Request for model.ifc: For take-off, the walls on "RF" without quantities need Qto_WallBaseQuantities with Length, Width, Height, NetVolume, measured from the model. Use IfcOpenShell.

First a look at what the model holds.

```python
import ifcopenshell
import ifcopenshell.util.element
import ifcopenshell.util.unit

model = ifcopenshell.open("model.ifc")
print(model.schema)
for unit_type in ("LENGTHUNIT", "AREAUNIT", "VOLUMEUNIT"):
    print(unit_type, ifcopenshell.util.unit.calculate_unit_scale(model, unit_type))
storey = next(s for s in model.by_type("IfcBuildingStorey") if s.Name == "RF")
walls = [e for e in ifcopenshell.util.element.get_decomposition(storey) if e.is_a("IfcWall")]
for e in sorted(walls, key=lambda e: e.id()):
    print(e.id(), e.is_a(), e.Name, list(ifcopenshell.util.element.get_psets(e, qtos_only=True)), sep=" | ")
```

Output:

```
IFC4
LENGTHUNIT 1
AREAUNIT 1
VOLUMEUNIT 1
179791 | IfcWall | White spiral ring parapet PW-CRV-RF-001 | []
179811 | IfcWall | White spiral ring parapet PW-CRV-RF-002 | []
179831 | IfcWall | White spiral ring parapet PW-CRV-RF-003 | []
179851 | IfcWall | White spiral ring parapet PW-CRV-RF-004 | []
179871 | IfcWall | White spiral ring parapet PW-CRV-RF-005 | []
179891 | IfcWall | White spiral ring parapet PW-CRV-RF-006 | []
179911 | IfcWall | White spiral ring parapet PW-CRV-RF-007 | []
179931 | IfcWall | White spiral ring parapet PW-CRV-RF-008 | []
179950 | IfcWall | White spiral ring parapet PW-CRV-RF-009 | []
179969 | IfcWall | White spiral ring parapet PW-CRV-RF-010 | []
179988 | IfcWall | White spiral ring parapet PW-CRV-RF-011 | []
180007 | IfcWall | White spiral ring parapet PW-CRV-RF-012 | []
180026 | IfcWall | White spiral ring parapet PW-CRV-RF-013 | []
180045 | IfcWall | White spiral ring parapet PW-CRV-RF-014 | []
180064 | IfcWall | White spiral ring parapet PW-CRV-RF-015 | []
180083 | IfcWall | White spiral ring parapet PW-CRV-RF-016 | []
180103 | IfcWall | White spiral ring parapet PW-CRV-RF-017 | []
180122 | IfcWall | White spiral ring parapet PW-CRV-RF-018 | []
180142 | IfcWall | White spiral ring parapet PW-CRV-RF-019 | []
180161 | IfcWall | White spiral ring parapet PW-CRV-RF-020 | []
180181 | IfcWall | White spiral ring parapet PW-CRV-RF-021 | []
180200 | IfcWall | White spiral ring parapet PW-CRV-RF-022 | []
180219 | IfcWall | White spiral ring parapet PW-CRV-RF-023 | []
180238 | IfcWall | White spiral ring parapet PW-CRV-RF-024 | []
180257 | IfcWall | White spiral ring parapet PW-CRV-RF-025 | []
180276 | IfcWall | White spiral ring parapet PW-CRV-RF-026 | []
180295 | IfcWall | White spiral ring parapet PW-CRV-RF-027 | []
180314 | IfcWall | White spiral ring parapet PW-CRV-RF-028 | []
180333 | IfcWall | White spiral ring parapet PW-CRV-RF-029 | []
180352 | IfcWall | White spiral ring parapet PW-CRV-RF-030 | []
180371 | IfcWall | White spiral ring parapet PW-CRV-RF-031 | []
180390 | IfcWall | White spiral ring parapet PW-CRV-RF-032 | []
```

```python
import ifcopenshell
import ifcopenshell.api.pset
import ifcopenshell.geom
import ifcopenshell.util.element
import ifcopenshell.util.shape
import ifcopenshell.util.unit

model = ifcopenshell.open("model.ifc")
unit_scale = ifcopenshell.util.unit.calculate_unit_scale(model)
volume_scale = ifcopenshell.util.unit.calculate_unit_scale(model, "VOLUMEUNIT")
settings = ifcopenshell.geom.settings()

storey = next(s for s in model.by_type("IfcBuildingStorey") if s.Name == "RF")
walls = [e for e in ifcopenshell.util.element.get_decomposition(storey) if e.is_a("IfcWall")]

for e in sorted(walls, key=lambda e: e.id()):
    if ifcopenshell.util.element.get_psets(e, qtos_only=True, should_inherit=False):
        continue
    # Geometry comes back in metres, in the element's own axes.
    shape = ifcopenshell.geom.create_shape(settings, e)
    values = {
        "Length": ifcopenshell.util.shape.get_x(shape.geometry) / unit_scale,
        "Width": ifcopenshell.util.shape.get_y(shape.geometry) / unit_scale,
        "Height": ifcopenshell.util.shape.get_z(shape.geometry) / unit_scale,
        "NetVolume": ifcopenshell.util.shape.get_volume(shape.geometry) / volume_scale,
    }
    qto = ifcopenshell.api.pset.add_qto(model, product=e, name="Qto_WallBaseQuantities")
    ifcopenshell.api.pset.edit_qto(model, qto=qto, properties=values)
    print(e.id(), {k: round(v, 3) for k, v in values.items()})

model.write("model_rev.ifc")
```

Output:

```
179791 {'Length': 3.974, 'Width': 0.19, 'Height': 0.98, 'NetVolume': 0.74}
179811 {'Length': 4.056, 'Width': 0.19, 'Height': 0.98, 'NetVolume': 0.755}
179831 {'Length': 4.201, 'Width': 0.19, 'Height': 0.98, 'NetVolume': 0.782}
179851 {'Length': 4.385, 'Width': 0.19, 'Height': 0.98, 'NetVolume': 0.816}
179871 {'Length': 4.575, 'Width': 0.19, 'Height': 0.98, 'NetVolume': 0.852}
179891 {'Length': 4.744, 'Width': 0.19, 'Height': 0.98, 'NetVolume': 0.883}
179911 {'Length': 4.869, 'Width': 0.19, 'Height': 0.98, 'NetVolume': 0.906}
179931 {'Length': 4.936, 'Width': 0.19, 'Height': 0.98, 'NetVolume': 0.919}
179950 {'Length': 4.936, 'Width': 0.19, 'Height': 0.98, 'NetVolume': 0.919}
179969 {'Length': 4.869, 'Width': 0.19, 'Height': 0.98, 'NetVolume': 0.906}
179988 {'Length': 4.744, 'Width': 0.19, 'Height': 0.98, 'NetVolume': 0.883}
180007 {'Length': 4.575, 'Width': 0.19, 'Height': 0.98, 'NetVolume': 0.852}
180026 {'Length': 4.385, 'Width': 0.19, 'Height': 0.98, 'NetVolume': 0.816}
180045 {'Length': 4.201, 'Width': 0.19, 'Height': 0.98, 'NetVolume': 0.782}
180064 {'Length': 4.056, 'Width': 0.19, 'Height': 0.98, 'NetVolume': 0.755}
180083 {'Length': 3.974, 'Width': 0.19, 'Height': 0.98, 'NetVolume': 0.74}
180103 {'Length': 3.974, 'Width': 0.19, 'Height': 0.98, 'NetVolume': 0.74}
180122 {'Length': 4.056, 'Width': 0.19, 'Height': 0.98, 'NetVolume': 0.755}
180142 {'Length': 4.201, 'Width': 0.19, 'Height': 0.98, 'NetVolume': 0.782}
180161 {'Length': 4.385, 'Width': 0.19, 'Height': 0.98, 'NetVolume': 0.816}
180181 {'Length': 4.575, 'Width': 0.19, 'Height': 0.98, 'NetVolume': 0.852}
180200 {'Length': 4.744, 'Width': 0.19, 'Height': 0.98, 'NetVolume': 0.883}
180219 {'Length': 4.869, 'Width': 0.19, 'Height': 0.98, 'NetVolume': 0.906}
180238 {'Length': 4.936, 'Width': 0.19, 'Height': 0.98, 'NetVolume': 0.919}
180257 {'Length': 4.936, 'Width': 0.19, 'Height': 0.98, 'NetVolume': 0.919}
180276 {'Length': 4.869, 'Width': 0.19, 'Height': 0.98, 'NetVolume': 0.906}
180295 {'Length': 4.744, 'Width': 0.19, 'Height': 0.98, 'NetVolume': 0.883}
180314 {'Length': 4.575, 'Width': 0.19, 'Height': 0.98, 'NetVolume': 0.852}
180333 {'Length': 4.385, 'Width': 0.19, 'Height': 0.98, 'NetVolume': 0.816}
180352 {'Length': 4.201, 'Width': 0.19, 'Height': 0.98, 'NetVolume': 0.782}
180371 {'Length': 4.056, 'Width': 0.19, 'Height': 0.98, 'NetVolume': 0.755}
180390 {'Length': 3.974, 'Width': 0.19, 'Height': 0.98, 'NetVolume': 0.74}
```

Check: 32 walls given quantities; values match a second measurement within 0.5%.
